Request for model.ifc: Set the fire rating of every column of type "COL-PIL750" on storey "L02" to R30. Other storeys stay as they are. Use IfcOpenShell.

First a look at what the model holds.

```python
import ifcopenshell
import ifcopenshell.util.element

model = ifcopenshell.open("model.ifc")
print(model.schema)
storey = next(s for s in model.by_type("IfcBuildingStorey") if s.Name == "L02")
columns = [e for e in ifcopenshell.util.element.get_decomposition(storey) if e.is_a("IfcColumn")]
seen = {}
for e in columns:
    element_type = ifcopenshell.util.element.get_type(e)
    key = (element_type.Name if element_type != e and element_type else None, ifcopenshell.util.element.get_pset(e, "Pset_ColumnCommon", "FireRating"))
    seen[key] = seen.get(key, 0) + 1
for (name, value), count in sorted(seen.items(), key=str):
    print(count, "x", name, "|", value)
```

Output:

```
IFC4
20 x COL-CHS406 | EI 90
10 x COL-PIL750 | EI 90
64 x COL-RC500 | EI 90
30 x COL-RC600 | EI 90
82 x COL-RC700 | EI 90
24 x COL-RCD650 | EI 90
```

```python
import ifcopenshell
import ifcopenshell.api.pset
import ifcopenshell.util.element

model = ifcopenshell.open("model.ifc")

storey = next(s for s in model.by_type("IfcBuildingStorey") if s.Name == "L02")
columns = [e for e in ifcopenshell.util.element.get_decomposition(storey) if e.is_a("IfcColumn")]

count = 0
for e in columns:
    element_type = ifcopenshell.util.element.get_type(e)
    if element_type in (None, e) or element_type.Name != "COL-PIL750":
        continue
    # add_pset returns the element's existing set when there is one.
    pset = ifcopenshell.api.pset.add_pset(model, product=e, name="Pset_ColumnCommon")
    ifcopenshell.api.pset.edit_pset(model, pset=pset, properties={"FireRating": "R30"})
    count += 1

print(count, "columns updated")

model.write("model-out.ifc")
```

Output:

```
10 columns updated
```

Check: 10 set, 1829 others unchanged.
